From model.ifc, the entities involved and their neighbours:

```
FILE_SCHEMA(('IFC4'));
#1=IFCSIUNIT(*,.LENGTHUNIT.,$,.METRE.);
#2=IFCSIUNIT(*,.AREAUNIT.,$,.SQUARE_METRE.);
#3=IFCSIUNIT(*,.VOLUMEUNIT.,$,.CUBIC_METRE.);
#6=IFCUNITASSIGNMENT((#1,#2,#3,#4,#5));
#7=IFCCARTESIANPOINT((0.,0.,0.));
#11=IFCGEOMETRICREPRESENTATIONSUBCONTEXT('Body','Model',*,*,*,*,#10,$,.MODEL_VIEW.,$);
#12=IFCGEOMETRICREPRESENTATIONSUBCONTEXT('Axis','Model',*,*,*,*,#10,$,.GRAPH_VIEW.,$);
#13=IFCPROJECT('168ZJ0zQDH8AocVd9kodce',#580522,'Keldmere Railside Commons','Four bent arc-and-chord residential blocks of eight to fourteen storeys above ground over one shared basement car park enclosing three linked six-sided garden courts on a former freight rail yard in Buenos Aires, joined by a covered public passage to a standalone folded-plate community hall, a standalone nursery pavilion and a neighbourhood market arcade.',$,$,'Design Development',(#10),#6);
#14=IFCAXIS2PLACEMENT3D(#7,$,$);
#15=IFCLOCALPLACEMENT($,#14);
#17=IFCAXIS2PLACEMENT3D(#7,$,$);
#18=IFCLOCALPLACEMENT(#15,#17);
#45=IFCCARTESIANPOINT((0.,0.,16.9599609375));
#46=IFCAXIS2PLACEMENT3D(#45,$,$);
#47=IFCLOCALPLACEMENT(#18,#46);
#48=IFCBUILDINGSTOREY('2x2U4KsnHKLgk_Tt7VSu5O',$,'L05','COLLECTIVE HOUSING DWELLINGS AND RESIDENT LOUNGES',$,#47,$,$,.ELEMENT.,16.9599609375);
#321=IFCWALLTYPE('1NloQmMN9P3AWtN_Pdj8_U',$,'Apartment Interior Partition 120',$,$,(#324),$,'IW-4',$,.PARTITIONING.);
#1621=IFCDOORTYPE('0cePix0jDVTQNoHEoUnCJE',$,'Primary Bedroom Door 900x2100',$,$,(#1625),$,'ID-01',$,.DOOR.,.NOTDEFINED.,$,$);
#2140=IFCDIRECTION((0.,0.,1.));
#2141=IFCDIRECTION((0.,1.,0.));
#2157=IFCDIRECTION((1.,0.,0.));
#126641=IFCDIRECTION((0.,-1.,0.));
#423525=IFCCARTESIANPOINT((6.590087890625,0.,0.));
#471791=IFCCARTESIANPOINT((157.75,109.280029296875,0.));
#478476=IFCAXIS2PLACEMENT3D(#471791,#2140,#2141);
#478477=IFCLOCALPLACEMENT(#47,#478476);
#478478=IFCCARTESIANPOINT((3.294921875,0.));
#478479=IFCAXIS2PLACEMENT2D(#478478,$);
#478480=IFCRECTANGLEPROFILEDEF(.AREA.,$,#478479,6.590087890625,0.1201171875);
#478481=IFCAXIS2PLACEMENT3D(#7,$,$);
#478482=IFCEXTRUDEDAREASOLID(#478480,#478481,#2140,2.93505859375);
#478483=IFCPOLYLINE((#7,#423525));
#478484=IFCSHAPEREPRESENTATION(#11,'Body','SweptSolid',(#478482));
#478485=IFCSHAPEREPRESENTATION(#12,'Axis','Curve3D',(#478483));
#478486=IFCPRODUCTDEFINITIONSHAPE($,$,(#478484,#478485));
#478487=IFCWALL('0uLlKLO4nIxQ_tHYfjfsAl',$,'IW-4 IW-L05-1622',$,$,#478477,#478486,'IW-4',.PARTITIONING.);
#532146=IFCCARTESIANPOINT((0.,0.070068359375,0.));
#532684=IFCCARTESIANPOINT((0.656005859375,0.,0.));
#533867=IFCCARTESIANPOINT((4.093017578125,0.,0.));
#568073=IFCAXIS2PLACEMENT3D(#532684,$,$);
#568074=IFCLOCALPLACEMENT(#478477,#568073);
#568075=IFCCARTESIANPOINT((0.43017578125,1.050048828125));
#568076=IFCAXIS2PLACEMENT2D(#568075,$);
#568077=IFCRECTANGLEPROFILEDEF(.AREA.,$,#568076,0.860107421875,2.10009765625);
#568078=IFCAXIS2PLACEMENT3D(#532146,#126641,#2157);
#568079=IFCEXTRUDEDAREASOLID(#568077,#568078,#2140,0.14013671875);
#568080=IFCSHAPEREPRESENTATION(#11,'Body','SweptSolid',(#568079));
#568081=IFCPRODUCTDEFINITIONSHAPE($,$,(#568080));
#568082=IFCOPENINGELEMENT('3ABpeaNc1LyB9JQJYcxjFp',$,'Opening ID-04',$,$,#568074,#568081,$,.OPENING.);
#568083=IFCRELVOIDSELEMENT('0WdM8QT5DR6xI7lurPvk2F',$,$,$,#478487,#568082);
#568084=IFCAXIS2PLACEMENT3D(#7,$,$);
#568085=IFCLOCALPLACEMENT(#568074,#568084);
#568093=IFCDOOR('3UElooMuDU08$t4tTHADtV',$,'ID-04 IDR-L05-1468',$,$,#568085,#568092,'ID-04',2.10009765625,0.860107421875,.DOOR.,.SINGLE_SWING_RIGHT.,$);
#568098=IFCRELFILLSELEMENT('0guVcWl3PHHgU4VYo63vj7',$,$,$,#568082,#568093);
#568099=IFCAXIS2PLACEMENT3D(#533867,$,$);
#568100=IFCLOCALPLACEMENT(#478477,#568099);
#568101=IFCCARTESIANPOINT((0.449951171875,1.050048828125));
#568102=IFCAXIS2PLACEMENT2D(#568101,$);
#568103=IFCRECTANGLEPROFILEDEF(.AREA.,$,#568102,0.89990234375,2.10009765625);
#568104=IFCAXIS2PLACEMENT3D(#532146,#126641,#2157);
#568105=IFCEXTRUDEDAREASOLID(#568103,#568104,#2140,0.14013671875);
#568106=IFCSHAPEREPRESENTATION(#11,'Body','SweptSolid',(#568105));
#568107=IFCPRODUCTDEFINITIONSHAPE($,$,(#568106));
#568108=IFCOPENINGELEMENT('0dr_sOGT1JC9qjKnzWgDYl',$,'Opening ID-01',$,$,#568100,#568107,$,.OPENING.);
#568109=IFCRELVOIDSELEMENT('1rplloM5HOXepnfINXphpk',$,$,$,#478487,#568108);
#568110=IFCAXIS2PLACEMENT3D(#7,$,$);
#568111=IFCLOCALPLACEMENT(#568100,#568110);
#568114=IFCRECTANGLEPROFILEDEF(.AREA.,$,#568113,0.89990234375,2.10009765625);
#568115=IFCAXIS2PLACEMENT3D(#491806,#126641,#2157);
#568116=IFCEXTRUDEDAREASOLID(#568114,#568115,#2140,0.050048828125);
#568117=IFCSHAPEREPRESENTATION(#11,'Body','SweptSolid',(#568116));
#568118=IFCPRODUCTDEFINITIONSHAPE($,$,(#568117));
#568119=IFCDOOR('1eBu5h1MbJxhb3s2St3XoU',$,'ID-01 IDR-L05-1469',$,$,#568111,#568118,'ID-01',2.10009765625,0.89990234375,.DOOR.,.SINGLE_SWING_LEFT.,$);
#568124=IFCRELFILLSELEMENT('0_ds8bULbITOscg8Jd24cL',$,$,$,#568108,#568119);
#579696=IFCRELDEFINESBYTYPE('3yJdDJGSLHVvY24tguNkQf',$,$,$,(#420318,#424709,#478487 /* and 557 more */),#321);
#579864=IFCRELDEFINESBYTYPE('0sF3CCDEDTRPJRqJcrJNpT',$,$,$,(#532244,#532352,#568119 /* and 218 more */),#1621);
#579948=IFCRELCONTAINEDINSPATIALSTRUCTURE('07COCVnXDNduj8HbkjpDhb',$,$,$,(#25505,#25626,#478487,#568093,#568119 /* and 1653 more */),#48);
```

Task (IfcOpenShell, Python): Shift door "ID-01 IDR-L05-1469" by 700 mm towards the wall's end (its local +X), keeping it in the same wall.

```python
import ifcopenshell
import ifcopenshell.api.geometry
import ifcopenshell.util.placement
import ifcopenshell.util.unit

model = ifcopenshell.open("model.ifc")
unit_scale = ifcopenshell.util.unit.calculate_unit_scale(model)

door = model.by_guid("1eBu5h1MbJxhb3s2St3XoU")
opening = door.FillsVoids[0].RelatingOpeningElement
wall = opening.VoidsElements[0].RelatingBuildingElement

wall_matrix = ifcopenshell.util.placement.get_local_placement(wall.ObjectPlacement)
shift = wall_matrix[:3, 0] * 0.7 / unit_scale
before = ifcopenshell.util.placement.get_local_placement(door.ObjectPlacement)[:3, 3].copy()

# The door is placed relative to its opening, so it follows when the opening moves.
matrix = ifcopenshell.util.placement.get_local_placement(opening.ObjectPlacement)
matrix[:3, 3] += shift
ifcopenshell.api.geometry.edit_object_placement(
    model, product=opening, matrix=matrix, is_si=False, should_transform_children=True
)

after = ifcopenshell.util.placement.get_local_placement(door.ObjectPlacement)[:3, 3]
print("door moved by", (after - before).round(3) + 0.0)

model.write("model-out.ifc")
```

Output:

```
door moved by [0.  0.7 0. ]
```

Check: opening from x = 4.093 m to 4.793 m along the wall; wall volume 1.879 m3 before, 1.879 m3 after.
